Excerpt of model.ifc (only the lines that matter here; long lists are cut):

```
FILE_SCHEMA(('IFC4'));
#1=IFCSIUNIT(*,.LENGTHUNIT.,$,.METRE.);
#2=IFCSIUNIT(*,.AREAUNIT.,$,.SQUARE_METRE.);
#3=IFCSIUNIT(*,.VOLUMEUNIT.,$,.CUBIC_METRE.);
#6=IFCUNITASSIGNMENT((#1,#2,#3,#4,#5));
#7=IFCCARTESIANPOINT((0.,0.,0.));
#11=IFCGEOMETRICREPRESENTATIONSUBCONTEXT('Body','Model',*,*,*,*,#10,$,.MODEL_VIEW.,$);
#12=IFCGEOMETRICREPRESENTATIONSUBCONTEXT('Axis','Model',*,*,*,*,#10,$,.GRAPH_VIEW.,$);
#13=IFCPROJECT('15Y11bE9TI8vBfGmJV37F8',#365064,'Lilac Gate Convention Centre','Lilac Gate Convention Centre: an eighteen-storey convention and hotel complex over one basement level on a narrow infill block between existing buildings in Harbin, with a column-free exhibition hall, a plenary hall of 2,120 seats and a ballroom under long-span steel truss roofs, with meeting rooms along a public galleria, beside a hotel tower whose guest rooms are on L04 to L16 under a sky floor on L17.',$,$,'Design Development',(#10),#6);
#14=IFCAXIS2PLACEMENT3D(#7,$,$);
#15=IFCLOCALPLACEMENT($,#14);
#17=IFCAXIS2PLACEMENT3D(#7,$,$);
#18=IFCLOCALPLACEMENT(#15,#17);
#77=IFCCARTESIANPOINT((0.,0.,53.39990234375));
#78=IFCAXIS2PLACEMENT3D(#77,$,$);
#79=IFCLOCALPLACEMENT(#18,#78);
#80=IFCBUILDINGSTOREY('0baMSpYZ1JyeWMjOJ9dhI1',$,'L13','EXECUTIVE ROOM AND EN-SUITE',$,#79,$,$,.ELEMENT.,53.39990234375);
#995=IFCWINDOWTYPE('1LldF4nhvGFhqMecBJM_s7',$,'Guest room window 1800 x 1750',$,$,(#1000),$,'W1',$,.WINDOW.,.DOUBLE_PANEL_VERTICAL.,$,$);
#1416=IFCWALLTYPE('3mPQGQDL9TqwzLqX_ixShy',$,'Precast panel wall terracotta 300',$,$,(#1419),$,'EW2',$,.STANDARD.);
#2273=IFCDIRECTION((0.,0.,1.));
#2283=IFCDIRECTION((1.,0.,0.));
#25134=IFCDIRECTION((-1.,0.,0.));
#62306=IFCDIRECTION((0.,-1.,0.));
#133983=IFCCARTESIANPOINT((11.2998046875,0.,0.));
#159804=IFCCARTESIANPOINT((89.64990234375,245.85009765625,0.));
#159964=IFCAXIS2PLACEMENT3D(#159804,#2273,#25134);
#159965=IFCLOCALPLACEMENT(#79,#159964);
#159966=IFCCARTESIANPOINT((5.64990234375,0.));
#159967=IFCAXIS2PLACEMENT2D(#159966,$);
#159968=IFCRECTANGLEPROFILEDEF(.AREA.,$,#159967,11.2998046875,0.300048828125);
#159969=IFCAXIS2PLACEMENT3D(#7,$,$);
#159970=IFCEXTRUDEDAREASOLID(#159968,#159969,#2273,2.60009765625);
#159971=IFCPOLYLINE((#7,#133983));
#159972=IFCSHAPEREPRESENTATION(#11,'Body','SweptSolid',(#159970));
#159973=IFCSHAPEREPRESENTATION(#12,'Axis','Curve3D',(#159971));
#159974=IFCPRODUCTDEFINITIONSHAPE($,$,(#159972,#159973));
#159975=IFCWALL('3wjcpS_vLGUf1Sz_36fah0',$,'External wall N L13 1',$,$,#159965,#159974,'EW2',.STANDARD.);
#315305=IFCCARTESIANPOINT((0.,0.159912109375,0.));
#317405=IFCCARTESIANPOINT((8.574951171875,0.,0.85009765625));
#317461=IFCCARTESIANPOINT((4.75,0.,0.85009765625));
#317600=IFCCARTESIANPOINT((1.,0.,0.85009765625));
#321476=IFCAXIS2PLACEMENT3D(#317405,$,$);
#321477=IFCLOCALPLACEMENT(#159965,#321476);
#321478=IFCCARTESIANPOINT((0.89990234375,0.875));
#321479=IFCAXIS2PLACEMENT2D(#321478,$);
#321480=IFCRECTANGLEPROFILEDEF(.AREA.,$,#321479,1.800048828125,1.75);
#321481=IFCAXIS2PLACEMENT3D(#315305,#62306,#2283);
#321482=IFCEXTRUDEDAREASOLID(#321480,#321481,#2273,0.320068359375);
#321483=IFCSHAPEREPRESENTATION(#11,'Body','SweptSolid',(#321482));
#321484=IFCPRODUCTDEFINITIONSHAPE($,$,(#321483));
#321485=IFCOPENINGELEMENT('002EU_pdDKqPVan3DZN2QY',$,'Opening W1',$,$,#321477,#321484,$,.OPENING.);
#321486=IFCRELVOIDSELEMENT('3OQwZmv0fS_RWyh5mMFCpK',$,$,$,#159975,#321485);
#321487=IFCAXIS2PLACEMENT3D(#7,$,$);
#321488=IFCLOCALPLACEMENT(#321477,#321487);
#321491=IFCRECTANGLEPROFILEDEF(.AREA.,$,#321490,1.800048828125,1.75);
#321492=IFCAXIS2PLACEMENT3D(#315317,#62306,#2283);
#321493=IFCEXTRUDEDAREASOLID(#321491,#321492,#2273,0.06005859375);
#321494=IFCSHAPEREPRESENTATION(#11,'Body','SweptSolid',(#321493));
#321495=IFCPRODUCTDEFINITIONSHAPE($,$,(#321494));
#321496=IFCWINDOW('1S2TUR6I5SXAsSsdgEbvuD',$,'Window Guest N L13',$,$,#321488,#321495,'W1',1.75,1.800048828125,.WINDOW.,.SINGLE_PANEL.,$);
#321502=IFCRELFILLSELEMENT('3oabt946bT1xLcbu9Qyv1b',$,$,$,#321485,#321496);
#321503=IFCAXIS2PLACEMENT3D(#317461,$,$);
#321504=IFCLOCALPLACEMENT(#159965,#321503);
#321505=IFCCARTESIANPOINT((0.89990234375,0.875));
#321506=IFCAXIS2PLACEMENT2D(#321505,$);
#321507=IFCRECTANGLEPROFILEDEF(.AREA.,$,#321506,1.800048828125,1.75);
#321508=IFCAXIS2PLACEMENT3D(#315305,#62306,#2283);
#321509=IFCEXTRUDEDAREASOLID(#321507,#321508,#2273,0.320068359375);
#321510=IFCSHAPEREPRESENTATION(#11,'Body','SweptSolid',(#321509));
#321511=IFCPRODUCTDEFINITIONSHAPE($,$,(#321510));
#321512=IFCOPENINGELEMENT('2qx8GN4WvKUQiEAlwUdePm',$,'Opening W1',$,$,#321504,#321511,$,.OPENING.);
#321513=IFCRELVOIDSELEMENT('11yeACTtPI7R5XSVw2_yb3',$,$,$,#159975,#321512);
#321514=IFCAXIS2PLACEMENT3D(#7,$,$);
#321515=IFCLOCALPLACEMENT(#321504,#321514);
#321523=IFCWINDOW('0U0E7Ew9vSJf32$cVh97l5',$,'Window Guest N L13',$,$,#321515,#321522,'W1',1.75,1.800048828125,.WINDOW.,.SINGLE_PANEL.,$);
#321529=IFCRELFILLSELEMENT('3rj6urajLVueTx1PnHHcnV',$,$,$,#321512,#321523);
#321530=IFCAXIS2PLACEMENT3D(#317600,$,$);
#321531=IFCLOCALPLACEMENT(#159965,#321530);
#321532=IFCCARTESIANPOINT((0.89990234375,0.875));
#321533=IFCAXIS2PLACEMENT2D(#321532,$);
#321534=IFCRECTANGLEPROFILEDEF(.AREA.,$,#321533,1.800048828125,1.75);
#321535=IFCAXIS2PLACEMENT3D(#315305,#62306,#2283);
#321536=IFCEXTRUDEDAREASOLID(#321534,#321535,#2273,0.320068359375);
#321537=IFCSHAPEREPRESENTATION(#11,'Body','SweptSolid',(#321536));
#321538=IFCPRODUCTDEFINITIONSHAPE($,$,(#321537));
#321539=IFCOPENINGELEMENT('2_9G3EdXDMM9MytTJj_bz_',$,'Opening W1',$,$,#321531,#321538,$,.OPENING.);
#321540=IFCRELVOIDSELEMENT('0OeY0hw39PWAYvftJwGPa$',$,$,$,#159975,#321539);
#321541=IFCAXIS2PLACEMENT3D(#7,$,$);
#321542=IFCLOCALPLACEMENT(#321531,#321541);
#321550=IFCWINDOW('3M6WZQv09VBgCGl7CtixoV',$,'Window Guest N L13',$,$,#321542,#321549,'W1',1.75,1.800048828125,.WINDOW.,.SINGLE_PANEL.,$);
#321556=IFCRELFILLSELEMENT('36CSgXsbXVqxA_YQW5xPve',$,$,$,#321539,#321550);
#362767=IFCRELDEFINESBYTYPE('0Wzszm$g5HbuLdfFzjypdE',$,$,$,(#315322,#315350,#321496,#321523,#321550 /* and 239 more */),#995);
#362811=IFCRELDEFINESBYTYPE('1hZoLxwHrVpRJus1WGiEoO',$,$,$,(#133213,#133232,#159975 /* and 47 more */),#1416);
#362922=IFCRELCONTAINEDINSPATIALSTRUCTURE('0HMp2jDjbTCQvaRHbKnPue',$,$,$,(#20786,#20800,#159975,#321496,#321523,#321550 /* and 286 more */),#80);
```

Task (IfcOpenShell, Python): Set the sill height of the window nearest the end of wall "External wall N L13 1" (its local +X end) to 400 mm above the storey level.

```python
import numpy as np
import ifcopenshell
import ifcopenshell.api.geometry
import ifcopenshell.geom
import ifcopenshell.util.element
import ifcopenshell.util.placement
import ifcopenshell.util.shape
import ifcopenshell.util.unit

model = ifcopenshell.open("model.ifc")
unit_scale = ifcopenshell.util.unit.calculate_unit_scale(model)

window = model.by_guid("1S2TUR6I5SXAsSsdgEbvuD")
opening = window.FillsVoids[0].RelatingOpeningElement
storey = ifcopenshell.util.element.get_container(window, ifc_class="IfcBuildingStorey")
level = ifcopenshell.util.placement.get_local_placement(storey.ObjectPlacement)[2, 3]

# The opening's origin need not be at the sill, so measure its lowest point.
shape = ifcopenshell.geom.create_shape(ifcopenshell.geom.settings(), opening)
bottom = ifcopenshell.util.shape.get_shape_bottom_elevation(shape, shape.geometry) / unit_scale
dz = level + 0.4 / unit_scale - bottom

shift = np.array([0.0, 0.0, dz])
# The window is placed relative to its opening, so it follows when the opening moves.
matrix = ifcopenshell.util.placement.get_local_placement(opening.ObjectPlacement)
matrix[:3, 3] += shift
ifcopenshell.api.geometry.edit_object_placement(
    model, product=opening, matrix=matrix, is_si=False, should_transform_children=True
)

print(f"moved by {dz * unit_scale:+.3f} m")

model.write("model_v2.ifc")
```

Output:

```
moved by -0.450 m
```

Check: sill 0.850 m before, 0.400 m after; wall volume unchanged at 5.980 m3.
